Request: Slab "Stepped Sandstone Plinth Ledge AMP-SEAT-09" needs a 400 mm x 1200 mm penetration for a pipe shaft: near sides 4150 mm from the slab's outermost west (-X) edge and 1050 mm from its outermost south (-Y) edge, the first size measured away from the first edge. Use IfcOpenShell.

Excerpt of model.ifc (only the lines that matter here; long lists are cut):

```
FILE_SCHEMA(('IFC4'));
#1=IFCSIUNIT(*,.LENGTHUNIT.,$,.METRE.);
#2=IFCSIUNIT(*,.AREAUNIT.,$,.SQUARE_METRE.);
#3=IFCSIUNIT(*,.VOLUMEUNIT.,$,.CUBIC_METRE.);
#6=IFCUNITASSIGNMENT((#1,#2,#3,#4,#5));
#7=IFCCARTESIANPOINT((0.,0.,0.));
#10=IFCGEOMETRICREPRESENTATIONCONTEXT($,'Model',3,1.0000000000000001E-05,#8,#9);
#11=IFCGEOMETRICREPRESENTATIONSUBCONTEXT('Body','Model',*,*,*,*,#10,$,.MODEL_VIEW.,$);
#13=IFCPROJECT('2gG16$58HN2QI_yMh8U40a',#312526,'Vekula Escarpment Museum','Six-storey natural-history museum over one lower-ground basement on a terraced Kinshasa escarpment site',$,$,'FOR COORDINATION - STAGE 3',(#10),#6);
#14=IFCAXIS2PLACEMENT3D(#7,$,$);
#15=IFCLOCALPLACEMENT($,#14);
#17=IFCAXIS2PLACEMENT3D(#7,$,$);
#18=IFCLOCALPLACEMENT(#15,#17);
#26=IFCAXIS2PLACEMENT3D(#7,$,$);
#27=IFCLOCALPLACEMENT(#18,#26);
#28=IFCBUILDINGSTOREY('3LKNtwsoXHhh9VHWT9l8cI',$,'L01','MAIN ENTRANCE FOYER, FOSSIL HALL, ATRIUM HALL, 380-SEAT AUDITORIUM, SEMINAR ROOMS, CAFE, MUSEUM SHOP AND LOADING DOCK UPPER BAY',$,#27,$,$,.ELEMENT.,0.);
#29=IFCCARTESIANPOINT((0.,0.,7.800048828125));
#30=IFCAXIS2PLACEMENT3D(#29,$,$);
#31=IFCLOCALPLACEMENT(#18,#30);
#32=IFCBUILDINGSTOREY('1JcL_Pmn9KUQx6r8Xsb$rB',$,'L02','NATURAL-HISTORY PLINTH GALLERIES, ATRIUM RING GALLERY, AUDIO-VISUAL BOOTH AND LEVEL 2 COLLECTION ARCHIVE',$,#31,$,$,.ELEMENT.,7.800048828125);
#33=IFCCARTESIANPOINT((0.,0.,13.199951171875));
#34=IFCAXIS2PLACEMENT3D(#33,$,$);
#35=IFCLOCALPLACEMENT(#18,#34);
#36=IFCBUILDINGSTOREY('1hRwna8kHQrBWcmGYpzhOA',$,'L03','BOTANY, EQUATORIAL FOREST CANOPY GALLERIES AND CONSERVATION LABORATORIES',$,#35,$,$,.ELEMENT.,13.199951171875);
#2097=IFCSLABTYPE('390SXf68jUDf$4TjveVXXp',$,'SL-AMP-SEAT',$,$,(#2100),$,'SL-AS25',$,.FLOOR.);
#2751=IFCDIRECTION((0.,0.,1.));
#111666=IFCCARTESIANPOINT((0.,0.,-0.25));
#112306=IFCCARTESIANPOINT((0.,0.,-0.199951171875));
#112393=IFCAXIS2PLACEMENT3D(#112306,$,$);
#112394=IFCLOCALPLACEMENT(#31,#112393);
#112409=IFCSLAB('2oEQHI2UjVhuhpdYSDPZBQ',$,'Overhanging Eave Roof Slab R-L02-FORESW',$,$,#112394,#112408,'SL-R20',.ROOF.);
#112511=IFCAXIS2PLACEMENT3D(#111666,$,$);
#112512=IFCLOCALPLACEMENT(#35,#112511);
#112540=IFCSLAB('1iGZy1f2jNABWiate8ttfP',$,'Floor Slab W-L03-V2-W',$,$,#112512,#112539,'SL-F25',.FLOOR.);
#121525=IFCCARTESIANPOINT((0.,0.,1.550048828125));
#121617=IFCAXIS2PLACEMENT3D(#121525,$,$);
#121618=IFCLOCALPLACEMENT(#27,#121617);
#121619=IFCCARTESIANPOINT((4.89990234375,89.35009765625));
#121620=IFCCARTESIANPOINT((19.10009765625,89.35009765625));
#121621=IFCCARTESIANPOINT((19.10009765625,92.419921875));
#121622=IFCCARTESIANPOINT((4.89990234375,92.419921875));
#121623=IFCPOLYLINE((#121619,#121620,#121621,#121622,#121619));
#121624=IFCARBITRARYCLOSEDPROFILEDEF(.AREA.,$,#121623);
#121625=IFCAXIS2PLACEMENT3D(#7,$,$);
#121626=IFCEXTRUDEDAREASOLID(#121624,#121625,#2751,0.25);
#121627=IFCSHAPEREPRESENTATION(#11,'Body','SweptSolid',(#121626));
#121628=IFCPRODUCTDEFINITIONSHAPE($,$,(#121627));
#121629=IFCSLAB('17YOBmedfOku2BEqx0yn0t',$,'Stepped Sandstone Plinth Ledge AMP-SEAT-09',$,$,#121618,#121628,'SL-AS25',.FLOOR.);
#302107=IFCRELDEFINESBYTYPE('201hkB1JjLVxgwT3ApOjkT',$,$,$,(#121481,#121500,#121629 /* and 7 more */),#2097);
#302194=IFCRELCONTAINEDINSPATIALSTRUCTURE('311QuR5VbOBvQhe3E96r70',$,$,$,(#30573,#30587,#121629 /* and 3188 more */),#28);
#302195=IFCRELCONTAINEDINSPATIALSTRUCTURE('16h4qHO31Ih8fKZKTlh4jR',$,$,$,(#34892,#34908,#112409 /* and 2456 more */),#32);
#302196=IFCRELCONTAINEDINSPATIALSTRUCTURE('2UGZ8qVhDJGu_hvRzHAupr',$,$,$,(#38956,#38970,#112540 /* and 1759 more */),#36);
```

```python
import numpy as np
import ifcopenshell
import ifcopenshell.api.feature
import ifcopenshell.api.geometry
import ifcopenshell.api.root
import ifcopenshell.geom
import ifcopenshell.util.placement
import ifcopenshell.util.representation
import ifcopenshell.util.shape
import ifcopenshell.util.unit

model = ifcopenshell.open("model.ifc")
unit_scale = ifcopenshell.util.unit.calculate_unit_scale(model)
settings = ifcopenshell.geom.settings()


def volume(element):
    """Net volume in cubic metres, openings subtracted."""
    shape = ifcopenshell.geom.create_shape(settings, element)
    return ifcopenshell.util.shape.get_volume(shape.geometry)


slab = model.by_guid("17YOBmedfOku2BEqx0yn0t")
before = volume(slab)

# Extent in the slab's own axes, in metres. The edges named are its -X and -Y sides.
slab_shape = ifcopenshell.geom.create_shape(settings, slab)
vertices = ifcopenshell.util.shape.get_vertices(slab_shape.geometry)
x_min, y_min, bottom = vertices.min(axis=0)
top = vertices[:, 2].max()

opening = ifcopenshell.api.root.create_entity(model, ifc_class="IfcOpeningElement", name="Pipe shaft opening", predefined_type="OPENING")
context = ifcopenshell.util.representation.get_context(model, "Model", "Body", "MODEL_VIEW")
width, depth = 0.4, 1.2
outline = [(0.0, 0.0), (width, 0.0), (width, depth), (0.0, depth), (0.0, 0.0)]
# Overshoot both faces by 50 mm so the cut is clean.
shape = ifcopenshell.api.geometry.add_slab_representation(
    model, context=context, depth=top - bottom + 0.1, polyline=outline
)
ifcopenshell.api.geometry.assign_representation(model, product=opening, representation=shape)

matrix = ifcopenshell.util.placement.get_local_placement(slab.ObjectPlacement)
matrix[:, 3] = matrix @ np.append(np.array([x_min + 4.15, y_min + 1.05, bottom - 0.05]) / unit_scale, 1.0)
ifcopenshell.api.geometry.edit_object_placement(model, product=opening, matrix=matrix, is_si=False)
ifcopenshell.api.feature.add_feature(model, feature=opening, element=slab)

after = volume(slab)

print(f"slab volume {before:.3f} -> {after:.3f} m3")

model.write("model_rev.ifc")
```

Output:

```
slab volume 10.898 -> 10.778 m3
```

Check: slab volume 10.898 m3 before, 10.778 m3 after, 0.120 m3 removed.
